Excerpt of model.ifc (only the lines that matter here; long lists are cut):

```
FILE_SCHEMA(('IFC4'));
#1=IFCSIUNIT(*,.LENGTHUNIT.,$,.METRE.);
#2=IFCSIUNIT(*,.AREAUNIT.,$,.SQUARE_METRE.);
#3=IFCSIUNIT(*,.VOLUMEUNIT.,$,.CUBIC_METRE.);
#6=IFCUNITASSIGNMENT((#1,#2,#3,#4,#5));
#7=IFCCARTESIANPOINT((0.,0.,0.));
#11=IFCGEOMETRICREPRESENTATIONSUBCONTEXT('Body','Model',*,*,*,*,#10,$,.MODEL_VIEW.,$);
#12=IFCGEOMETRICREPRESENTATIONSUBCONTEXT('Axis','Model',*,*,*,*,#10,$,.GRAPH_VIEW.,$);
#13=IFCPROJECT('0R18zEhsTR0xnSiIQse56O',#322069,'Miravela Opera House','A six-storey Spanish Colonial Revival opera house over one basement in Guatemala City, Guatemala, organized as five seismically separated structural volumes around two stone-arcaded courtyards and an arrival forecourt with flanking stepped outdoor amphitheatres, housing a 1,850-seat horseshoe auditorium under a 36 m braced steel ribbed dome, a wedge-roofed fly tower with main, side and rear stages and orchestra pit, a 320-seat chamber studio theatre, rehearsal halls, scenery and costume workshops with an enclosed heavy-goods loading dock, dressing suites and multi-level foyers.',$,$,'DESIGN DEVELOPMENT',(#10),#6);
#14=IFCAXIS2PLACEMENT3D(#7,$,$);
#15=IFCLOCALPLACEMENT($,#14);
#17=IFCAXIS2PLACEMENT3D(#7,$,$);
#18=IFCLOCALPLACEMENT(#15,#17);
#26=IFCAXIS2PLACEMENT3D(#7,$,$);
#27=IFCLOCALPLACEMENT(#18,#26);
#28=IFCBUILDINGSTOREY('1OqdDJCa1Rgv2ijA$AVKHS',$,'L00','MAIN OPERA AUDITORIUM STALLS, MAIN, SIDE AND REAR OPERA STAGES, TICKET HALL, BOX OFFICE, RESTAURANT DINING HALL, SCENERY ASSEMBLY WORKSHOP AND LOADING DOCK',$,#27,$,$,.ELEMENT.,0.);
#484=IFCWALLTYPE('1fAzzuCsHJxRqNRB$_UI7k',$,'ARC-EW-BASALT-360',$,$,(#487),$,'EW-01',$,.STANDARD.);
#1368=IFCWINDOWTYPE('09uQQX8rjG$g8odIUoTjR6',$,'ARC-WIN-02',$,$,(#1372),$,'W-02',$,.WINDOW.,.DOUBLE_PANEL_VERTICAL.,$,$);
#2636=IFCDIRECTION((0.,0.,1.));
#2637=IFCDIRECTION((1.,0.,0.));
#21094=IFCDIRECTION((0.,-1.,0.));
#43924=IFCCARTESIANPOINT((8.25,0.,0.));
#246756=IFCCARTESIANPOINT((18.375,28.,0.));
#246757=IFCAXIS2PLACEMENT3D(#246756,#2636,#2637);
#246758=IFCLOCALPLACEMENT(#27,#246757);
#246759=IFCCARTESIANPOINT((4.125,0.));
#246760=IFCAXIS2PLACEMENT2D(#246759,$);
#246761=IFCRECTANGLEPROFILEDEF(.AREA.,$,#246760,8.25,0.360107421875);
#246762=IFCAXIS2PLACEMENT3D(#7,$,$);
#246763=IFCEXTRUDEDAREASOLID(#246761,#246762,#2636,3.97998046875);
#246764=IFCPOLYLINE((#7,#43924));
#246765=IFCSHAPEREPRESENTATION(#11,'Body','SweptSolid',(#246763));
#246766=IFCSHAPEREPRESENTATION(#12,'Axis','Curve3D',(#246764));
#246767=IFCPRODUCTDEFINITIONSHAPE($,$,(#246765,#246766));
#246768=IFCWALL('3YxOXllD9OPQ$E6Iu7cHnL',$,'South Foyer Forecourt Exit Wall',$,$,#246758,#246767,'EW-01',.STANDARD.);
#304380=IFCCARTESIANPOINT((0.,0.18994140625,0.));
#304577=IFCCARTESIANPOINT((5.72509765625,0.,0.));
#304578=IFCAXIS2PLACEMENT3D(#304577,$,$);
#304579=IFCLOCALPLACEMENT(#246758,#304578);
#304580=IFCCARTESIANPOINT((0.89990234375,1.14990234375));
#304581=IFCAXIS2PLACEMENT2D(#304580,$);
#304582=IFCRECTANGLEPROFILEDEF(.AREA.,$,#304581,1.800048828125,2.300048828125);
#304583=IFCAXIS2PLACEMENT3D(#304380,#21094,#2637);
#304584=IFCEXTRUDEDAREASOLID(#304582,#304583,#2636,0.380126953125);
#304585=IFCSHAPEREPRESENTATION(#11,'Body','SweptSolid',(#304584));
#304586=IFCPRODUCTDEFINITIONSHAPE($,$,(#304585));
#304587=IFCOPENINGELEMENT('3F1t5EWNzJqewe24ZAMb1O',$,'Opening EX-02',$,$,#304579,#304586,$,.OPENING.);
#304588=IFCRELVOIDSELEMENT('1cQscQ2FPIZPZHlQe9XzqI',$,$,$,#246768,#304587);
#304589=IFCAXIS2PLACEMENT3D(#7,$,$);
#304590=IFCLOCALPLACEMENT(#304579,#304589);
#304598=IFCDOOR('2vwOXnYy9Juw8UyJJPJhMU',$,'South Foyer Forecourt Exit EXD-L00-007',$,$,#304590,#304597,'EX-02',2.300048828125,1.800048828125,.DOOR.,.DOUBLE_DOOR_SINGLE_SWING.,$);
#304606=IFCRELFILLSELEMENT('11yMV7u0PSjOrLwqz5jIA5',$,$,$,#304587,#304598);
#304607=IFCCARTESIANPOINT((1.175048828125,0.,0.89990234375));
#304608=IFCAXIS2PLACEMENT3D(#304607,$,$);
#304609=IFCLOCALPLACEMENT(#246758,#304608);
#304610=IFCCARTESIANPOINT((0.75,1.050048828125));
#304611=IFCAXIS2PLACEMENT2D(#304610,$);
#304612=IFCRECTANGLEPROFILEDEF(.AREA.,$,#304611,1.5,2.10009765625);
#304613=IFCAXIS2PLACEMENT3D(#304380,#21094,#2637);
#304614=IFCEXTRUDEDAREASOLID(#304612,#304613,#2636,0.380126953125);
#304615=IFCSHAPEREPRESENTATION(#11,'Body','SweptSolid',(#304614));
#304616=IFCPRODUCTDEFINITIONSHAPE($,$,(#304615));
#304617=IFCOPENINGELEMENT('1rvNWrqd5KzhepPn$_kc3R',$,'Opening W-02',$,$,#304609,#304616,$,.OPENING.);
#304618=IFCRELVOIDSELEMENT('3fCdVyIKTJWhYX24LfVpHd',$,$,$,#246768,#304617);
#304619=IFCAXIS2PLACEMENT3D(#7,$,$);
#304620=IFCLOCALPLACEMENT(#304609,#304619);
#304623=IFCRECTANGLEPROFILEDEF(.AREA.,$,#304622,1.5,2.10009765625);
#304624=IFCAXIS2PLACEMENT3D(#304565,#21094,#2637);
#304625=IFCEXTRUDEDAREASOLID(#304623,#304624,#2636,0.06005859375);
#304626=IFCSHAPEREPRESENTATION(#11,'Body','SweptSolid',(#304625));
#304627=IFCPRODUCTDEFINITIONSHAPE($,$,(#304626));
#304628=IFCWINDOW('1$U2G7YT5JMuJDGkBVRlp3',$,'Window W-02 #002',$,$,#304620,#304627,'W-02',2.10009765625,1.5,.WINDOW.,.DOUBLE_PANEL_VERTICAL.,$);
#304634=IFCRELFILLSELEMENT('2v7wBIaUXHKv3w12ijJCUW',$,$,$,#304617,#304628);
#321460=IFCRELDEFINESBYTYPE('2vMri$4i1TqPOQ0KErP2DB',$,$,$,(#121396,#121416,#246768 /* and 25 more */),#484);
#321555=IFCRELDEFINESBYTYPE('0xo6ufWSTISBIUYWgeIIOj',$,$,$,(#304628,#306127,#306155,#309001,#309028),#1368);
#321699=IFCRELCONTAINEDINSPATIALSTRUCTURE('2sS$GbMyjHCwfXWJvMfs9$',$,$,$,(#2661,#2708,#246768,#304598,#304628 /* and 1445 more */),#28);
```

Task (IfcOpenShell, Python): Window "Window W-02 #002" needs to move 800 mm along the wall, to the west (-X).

```python
import ifcopenshell
import ifcopenshell.api.geometry
import ifcopenshell.util.placement

model = ifcopenshell.open("model.ifc")

window = model.by_guid("1$U2G7YT5JMuJDGkBVRlp3")
opening = window.FillsVoids[0].RelatingOpeningElement
wall = opening.VoidsElements[0].RelatingBuildingElement

wall_matrix = ifcopenshell.util.placement.get_local_placement(wall.ObjectPlacement)
shift = wall_matrix[:3, 0] * -0.8
before = ifcopenshell.util.placement.get_local_placement(window.ObjectPlacement)[:3, 3].copy()

# The window is placed relative to its opening, so it follows when the opening moves.
matrix = ifcopenshell.util.placement.get_local_placement(opening.ObjectPlacement)
matrix[:3, 3] += shift
ifcopenshell.api.geometry.edit_object_placement(
    model, product=opening, matrix=matrix, is_si=False, should_transform_children=True
)

after = ifcopenshell.util.placement.get_local_placement(window.ObjectPlacement)[:3, 3]
print("window moved by", (after - before).round(3) + 0.0)

model.write("model_edited.ifc")
```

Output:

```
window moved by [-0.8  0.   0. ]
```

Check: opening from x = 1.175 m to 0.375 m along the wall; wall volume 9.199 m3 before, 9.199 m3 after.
